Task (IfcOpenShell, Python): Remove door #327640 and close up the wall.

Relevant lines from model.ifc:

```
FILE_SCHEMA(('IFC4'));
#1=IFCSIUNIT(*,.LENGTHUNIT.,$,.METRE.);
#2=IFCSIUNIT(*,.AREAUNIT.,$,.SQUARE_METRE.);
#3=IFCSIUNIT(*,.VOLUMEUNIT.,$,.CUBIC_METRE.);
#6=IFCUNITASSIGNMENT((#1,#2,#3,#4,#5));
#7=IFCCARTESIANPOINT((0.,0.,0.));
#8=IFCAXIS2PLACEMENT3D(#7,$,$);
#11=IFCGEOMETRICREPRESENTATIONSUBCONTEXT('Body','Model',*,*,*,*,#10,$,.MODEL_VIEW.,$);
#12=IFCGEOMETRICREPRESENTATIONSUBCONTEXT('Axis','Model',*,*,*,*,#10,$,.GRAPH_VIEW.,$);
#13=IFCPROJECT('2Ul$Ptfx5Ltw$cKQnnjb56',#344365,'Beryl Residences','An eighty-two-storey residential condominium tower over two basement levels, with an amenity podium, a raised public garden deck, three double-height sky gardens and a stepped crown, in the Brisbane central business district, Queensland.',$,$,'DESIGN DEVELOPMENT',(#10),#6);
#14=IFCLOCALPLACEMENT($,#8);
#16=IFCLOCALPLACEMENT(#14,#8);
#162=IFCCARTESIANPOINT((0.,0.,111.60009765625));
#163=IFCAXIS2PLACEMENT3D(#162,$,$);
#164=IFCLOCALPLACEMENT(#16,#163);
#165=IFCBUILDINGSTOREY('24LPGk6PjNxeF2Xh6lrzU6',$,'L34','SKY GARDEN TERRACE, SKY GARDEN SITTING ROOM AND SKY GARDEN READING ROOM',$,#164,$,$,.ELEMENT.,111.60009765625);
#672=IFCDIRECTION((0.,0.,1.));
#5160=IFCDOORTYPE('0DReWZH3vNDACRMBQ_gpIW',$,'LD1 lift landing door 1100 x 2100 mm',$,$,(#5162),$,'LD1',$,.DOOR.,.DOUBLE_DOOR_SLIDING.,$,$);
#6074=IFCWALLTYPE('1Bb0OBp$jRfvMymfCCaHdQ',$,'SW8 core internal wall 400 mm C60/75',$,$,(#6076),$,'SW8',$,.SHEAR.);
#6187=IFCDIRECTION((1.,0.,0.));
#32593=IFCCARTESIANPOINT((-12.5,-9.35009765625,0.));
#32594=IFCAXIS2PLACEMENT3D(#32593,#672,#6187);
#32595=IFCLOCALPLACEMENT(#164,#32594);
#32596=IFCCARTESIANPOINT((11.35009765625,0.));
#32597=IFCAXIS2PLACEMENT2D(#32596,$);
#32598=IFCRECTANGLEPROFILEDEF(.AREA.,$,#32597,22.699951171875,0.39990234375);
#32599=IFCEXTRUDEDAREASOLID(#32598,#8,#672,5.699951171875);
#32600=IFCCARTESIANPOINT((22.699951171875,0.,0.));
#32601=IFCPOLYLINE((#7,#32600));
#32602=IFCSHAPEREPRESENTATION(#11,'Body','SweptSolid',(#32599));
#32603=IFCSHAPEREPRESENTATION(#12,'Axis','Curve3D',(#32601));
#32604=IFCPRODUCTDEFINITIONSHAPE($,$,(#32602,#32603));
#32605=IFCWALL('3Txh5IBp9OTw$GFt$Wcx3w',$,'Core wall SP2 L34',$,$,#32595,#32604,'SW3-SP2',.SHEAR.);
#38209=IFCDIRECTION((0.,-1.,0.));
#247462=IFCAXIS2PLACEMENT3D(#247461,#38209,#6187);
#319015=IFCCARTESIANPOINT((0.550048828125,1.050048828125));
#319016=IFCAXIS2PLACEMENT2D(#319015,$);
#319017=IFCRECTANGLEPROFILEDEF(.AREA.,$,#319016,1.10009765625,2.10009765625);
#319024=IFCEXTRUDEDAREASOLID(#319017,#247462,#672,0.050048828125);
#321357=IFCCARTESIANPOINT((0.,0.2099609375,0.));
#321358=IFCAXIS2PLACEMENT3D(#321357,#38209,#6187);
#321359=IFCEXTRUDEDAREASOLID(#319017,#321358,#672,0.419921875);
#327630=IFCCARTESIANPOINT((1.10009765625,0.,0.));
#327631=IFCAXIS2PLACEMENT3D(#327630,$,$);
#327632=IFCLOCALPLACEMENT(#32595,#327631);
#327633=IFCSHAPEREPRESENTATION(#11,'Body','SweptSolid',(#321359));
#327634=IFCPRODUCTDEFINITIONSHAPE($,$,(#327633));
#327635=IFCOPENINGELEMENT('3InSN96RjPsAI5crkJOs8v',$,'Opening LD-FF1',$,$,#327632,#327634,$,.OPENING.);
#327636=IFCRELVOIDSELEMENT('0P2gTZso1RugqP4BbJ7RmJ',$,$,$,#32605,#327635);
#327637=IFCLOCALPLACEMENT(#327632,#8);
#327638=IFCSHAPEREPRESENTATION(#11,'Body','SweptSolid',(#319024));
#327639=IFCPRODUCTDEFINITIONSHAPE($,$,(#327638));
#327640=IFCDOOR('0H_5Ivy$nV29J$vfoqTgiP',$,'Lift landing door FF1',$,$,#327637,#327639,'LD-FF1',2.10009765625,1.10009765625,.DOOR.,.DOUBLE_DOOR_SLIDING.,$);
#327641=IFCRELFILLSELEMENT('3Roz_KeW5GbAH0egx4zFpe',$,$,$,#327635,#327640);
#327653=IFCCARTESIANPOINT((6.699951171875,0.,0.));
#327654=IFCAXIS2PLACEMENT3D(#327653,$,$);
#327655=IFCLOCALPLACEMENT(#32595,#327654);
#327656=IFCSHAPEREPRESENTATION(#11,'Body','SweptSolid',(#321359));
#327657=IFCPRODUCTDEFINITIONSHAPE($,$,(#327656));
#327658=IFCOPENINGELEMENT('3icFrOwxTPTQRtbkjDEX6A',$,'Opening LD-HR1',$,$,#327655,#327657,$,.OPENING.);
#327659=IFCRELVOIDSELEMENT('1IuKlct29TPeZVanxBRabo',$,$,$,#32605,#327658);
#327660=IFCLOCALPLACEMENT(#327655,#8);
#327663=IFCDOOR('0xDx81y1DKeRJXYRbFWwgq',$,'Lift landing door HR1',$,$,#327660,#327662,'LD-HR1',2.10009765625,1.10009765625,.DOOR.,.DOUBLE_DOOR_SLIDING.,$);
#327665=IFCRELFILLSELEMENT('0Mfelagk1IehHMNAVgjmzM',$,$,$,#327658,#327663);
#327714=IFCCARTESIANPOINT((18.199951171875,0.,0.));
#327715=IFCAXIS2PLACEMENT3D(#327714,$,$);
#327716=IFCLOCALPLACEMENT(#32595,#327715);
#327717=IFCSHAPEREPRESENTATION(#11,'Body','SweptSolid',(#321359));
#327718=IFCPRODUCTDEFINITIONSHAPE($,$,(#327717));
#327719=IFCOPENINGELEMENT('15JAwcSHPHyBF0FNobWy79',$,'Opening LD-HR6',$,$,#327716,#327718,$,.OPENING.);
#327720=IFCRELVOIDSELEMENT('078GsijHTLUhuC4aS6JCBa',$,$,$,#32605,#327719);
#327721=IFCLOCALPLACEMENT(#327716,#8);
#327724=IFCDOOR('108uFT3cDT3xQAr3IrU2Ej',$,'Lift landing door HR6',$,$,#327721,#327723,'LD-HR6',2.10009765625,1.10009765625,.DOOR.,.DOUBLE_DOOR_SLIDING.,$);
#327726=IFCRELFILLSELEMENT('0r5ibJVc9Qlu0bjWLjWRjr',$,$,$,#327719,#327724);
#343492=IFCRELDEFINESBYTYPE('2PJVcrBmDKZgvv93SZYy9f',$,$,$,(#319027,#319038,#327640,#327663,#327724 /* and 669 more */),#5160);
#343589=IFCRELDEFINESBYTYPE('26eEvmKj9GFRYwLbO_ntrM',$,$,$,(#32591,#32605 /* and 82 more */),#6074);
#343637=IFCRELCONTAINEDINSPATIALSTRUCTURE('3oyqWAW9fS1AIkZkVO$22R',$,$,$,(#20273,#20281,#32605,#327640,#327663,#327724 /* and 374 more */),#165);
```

```python
import ifcopenshell
import ifcopenshell.api.feature
import ifcopenshell.api.root
import ifcopenshell.geom
import ifcopenshell.util.shape

model = ifcopenshell.open("model.ifc")
settings = ifcopenshell.geom.settings()


def volume(element):
    """Net volume in cubic metres, openings subtracted."""
    shape = ifcopenshell.geom.create_shape(settings, element)
    return ifcopenshell.util.shape.get_volume(shape.geometry)


door = model.by_id(327640)
opening = door.FillsVoids[0].RelatingOpeningElement
wall = opening.VoidsElements[0].RelatingBuildingElement
before = volume(wall)

ifcopenshell.api.root.remove_product(model, product=door)
ifcopenshell.api.feature.remove_feature(model, feature=opening)

after = volume(wall)

print(f"wall volume {before:.3f} -> {after:.3f} m3")

model.write("model_edited.ifc")
```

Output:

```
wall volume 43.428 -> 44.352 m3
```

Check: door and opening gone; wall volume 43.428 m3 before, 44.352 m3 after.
